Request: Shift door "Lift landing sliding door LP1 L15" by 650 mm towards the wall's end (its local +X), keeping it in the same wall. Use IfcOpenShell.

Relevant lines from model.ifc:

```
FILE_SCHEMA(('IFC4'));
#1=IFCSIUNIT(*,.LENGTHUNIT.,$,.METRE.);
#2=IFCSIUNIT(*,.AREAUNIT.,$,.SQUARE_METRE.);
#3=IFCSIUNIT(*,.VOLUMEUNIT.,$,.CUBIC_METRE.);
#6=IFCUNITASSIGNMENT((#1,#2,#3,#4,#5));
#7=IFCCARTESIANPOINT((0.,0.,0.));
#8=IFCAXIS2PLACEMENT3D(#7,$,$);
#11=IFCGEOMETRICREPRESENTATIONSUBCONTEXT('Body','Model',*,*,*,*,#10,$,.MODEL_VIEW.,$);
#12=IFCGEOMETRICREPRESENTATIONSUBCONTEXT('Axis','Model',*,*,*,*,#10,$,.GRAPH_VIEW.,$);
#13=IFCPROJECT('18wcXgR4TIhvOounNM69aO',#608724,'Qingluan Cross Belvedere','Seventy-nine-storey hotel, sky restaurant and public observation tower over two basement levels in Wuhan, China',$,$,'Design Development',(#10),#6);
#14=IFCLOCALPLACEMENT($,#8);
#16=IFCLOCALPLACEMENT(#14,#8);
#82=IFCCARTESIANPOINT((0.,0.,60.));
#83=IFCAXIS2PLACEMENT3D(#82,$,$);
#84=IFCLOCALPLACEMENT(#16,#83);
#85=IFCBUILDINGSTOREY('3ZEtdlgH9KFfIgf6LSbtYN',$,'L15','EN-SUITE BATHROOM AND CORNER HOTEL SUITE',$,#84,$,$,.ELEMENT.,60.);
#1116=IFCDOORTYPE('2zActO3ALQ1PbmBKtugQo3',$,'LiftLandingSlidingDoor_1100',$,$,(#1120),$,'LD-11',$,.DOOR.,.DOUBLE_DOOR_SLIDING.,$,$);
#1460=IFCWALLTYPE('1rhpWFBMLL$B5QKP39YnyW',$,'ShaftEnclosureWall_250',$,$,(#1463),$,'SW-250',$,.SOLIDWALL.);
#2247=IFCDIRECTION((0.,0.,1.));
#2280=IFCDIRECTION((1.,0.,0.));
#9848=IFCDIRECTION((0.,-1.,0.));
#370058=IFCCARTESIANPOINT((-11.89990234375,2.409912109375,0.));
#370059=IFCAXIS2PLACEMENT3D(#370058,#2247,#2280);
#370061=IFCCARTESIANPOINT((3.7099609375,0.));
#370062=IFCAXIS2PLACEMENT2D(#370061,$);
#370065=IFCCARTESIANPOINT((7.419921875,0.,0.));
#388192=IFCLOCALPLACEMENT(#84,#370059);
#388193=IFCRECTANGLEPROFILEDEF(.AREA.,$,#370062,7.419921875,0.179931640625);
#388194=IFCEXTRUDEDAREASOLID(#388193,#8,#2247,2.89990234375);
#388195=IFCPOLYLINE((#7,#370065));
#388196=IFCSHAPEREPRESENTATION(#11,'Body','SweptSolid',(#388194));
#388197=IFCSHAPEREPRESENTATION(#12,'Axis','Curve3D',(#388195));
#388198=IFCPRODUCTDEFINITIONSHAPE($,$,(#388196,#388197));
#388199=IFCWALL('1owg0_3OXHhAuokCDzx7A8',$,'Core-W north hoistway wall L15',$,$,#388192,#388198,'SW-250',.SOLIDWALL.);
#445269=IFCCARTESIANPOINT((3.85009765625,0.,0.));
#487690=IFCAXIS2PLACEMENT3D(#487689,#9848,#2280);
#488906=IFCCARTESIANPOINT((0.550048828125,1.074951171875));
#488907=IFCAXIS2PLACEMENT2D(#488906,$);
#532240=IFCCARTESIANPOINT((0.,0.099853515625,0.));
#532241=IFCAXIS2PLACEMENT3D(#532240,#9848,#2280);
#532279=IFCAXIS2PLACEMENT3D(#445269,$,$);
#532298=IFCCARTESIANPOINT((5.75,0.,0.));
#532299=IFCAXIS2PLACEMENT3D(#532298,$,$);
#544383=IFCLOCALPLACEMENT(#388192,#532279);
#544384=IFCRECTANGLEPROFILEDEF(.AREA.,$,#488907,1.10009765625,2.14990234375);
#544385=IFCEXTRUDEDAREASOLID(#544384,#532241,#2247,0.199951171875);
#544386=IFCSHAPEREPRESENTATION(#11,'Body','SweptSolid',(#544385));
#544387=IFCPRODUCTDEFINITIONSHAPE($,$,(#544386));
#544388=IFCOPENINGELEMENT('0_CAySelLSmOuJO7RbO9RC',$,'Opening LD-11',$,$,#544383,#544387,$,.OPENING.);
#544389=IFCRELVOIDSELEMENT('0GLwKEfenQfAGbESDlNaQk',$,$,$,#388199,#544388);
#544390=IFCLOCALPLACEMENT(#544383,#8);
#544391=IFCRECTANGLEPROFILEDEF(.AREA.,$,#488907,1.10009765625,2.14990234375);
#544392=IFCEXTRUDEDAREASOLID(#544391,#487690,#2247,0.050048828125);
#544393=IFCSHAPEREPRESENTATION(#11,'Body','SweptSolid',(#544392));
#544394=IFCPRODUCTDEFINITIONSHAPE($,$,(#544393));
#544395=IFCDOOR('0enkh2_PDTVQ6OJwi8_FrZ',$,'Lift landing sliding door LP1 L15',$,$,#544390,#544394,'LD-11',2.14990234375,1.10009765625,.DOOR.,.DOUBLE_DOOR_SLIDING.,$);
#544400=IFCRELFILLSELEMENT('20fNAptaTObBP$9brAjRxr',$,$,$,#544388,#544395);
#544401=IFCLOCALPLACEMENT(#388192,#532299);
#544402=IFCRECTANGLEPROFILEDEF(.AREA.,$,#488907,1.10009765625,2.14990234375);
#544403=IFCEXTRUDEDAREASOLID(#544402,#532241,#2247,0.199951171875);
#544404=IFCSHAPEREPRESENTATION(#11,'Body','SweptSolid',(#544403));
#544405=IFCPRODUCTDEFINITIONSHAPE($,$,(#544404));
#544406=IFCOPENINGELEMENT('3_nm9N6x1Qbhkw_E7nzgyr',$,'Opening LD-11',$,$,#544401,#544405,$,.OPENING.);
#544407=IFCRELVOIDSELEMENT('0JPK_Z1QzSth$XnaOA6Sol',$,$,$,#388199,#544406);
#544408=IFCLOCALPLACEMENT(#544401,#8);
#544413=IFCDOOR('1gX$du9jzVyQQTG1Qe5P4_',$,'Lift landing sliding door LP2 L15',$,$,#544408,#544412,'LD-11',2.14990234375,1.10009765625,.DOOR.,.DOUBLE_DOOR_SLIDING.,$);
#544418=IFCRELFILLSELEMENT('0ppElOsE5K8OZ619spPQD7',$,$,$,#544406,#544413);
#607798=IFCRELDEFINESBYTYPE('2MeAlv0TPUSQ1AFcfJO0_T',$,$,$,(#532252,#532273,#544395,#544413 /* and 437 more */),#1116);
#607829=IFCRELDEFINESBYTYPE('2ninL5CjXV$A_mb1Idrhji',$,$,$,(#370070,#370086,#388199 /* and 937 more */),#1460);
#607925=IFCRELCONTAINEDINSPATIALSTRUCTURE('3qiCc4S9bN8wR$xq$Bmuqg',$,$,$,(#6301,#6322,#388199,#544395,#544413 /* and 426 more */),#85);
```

```python
import ifcopenshell
import ifcopenshell.api.geometry
import ifcopenshell.util.placement

model = ifcopenshell.open("model.ifc")

door = model.by_id(544395)
opening = door.FillsVoids[0].RelatingOpeningElement
wall = opening.VoidsElements[0].RelatingBuildingElement

wall_matrix = ifcopenshell.util.placement.get_local_placement(wall.ObjectPlacement)
shift = wall_matrix[:3, 0] * 0.65
before = ifcopenshell.util.placement.get_local_placement(door.ObjectPlacement)[:3, 3].copy()

# The door is placed relative to its opening, so it follows when the opening moves.
matrix = ifcopenshell.util.placement.get_local_placement(opening.ObjectPlacement)
matrix[:3, 3] += shift
ifcopenshell.api.geometry.edit_object_placement(
    model, product=opening, matrix=matrix, is_si=False, should_transform_children=True
)

after = ifcopenshell.util.placement.get_local_placement(door.ObjectPlacement)[:3, 3]
print("door moved by", (after - before).round(3) + 0.0)

model.write("model_updated.ifc")
```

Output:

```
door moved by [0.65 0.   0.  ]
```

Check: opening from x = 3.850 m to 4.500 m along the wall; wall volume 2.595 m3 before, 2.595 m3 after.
